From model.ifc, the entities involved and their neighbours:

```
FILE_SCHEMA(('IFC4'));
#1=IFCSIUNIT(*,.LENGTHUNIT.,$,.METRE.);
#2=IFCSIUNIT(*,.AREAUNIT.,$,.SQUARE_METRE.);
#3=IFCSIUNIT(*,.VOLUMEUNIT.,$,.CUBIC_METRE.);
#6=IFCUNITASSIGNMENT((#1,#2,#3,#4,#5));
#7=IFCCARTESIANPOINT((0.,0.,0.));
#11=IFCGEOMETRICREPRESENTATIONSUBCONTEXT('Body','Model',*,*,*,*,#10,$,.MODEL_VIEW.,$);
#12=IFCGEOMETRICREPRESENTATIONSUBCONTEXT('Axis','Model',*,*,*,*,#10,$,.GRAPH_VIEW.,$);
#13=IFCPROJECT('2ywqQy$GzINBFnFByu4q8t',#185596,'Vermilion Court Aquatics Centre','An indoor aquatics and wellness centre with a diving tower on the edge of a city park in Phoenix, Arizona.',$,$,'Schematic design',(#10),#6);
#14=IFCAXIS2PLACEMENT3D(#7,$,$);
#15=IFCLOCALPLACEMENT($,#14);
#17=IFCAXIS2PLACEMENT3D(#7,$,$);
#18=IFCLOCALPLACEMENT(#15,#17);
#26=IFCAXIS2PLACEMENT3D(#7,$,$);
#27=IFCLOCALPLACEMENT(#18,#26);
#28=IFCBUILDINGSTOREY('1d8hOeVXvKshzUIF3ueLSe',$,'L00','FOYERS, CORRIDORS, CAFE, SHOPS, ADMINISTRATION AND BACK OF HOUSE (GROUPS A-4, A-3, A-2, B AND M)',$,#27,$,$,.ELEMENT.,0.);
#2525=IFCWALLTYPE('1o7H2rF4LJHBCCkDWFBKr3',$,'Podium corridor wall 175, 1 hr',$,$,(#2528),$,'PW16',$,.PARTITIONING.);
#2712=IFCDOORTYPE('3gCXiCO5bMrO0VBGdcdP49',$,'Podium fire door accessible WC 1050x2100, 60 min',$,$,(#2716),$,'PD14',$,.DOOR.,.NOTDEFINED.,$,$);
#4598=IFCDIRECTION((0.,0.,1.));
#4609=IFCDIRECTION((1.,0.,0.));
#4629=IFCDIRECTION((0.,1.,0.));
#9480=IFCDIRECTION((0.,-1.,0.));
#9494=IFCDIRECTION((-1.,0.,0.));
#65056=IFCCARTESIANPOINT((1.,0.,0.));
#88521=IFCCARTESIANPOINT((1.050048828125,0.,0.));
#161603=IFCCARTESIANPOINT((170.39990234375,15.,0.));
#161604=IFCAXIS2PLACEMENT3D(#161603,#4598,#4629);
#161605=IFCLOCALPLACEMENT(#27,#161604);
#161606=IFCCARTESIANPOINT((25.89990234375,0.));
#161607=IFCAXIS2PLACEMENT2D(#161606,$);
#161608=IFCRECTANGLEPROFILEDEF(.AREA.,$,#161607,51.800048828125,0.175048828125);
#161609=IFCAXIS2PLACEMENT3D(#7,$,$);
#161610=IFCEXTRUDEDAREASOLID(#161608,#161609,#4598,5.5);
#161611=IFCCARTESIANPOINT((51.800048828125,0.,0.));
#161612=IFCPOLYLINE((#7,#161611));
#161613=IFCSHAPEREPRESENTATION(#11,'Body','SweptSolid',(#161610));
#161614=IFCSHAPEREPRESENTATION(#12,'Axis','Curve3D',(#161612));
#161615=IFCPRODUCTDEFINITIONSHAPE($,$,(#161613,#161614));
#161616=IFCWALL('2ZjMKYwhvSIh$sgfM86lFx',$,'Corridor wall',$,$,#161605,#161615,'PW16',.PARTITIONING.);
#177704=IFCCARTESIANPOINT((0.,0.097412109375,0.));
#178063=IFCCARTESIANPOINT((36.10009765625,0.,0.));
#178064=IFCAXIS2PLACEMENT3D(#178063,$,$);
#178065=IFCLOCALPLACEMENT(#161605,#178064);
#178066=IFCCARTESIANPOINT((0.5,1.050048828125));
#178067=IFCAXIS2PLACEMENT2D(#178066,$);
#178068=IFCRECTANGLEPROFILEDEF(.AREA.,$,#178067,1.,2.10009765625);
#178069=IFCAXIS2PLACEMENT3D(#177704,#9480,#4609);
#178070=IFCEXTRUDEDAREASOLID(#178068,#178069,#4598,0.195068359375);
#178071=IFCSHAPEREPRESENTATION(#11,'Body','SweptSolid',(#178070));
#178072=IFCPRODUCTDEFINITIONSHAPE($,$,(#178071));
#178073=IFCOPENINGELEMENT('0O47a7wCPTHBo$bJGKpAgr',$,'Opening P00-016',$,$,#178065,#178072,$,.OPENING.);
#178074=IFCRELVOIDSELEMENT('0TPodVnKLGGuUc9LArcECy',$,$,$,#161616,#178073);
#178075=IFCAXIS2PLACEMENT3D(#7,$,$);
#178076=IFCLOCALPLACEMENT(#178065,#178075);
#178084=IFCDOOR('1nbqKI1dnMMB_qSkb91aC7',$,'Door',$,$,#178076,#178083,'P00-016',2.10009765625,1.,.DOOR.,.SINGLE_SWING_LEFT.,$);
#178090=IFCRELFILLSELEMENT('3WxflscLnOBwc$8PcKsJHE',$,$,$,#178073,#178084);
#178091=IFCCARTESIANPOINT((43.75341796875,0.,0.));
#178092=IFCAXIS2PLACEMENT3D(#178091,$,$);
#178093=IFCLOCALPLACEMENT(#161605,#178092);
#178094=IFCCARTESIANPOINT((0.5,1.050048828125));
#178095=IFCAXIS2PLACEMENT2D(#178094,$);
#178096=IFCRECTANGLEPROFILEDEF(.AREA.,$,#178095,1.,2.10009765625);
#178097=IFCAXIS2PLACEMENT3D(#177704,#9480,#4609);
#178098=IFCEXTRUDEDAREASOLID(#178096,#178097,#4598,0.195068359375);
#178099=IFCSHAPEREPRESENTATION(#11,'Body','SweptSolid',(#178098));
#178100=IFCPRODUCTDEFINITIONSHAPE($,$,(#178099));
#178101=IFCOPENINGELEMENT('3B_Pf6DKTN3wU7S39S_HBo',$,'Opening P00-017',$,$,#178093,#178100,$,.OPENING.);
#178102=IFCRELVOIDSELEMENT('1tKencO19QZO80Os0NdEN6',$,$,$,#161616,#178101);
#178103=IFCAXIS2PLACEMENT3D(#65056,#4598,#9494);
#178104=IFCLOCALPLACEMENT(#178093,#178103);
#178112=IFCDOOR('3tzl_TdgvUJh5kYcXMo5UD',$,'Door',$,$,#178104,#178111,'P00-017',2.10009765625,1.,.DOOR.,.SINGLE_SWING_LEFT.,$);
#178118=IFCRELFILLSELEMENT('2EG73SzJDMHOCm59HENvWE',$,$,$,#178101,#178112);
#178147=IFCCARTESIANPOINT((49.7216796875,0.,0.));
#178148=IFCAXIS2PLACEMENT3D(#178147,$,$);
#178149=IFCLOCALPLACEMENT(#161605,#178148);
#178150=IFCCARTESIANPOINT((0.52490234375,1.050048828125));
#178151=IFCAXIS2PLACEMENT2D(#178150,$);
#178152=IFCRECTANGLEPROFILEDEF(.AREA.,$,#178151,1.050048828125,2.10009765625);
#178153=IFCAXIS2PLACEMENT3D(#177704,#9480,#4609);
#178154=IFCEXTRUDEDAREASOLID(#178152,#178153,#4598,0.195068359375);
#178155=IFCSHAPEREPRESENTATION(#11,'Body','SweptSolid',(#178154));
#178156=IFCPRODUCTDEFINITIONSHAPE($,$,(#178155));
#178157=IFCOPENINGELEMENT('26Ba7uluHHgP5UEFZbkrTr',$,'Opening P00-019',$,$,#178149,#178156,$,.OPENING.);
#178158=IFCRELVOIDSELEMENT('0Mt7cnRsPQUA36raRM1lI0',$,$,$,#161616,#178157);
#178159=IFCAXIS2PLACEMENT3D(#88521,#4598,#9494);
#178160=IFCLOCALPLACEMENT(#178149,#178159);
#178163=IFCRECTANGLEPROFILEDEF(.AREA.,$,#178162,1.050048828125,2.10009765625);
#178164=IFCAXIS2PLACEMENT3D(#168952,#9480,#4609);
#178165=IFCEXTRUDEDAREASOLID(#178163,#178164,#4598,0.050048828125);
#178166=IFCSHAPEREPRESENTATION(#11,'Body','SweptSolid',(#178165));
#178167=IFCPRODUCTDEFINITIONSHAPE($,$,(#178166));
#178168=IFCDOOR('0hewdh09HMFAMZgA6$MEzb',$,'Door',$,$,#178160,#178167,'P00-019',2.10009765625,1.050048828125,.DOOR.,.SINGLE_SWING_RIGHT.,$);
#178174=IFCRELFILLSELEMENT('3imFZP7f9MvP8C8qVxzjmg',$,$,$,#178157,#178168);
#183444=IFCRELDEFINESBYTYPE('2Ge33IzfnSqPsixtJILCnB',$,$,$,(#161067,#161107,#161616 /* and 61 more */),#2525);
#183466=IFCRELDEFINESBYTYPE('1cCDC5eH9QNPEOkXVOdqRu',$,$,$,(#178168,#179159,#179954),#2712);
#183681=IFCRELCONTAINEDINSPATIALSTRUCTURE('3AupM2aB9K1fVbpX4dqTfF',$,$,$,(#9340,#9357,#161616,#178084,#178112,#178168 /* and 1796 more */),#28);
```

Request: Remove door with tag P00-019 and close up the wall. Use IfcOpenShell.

```python
import ifcopenshell
import ifcopenshell.api.feature
import ifcopenshell.api.root
import ifcopenshell.geom
import ifcopenshell.util.shape

model = ifcopenshell.open("model.ifc")
settings = ifcopenshell.geom.settings()


def volume(element):
    """Net volume in cubic metres, openings subtracted."""
    shape = ifcopenshell.geom.create_shape(settings, element)
    return ifcopenshell.util.shape.get_volume(shape.geometry)


door = model.by_id(178168)
opening = door.FillsVoids[0].RelatingOpeningElement
wall = opening.VoidsElements[0].RelatingBuildingElement
before = volume(wall)

ifcopenshell.api.root.remove_product(model, product=door)
ifcopenshell.api.feature.remove_feature(model, feature=opening)

after = volume(wall)

print(f"wall volume {before:.3f} -> {after:.3f} m3")

model.write("model_updated.ifc")
```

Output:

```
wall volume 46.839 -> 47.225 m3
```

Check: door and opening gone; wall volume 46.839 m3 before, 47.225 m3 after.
